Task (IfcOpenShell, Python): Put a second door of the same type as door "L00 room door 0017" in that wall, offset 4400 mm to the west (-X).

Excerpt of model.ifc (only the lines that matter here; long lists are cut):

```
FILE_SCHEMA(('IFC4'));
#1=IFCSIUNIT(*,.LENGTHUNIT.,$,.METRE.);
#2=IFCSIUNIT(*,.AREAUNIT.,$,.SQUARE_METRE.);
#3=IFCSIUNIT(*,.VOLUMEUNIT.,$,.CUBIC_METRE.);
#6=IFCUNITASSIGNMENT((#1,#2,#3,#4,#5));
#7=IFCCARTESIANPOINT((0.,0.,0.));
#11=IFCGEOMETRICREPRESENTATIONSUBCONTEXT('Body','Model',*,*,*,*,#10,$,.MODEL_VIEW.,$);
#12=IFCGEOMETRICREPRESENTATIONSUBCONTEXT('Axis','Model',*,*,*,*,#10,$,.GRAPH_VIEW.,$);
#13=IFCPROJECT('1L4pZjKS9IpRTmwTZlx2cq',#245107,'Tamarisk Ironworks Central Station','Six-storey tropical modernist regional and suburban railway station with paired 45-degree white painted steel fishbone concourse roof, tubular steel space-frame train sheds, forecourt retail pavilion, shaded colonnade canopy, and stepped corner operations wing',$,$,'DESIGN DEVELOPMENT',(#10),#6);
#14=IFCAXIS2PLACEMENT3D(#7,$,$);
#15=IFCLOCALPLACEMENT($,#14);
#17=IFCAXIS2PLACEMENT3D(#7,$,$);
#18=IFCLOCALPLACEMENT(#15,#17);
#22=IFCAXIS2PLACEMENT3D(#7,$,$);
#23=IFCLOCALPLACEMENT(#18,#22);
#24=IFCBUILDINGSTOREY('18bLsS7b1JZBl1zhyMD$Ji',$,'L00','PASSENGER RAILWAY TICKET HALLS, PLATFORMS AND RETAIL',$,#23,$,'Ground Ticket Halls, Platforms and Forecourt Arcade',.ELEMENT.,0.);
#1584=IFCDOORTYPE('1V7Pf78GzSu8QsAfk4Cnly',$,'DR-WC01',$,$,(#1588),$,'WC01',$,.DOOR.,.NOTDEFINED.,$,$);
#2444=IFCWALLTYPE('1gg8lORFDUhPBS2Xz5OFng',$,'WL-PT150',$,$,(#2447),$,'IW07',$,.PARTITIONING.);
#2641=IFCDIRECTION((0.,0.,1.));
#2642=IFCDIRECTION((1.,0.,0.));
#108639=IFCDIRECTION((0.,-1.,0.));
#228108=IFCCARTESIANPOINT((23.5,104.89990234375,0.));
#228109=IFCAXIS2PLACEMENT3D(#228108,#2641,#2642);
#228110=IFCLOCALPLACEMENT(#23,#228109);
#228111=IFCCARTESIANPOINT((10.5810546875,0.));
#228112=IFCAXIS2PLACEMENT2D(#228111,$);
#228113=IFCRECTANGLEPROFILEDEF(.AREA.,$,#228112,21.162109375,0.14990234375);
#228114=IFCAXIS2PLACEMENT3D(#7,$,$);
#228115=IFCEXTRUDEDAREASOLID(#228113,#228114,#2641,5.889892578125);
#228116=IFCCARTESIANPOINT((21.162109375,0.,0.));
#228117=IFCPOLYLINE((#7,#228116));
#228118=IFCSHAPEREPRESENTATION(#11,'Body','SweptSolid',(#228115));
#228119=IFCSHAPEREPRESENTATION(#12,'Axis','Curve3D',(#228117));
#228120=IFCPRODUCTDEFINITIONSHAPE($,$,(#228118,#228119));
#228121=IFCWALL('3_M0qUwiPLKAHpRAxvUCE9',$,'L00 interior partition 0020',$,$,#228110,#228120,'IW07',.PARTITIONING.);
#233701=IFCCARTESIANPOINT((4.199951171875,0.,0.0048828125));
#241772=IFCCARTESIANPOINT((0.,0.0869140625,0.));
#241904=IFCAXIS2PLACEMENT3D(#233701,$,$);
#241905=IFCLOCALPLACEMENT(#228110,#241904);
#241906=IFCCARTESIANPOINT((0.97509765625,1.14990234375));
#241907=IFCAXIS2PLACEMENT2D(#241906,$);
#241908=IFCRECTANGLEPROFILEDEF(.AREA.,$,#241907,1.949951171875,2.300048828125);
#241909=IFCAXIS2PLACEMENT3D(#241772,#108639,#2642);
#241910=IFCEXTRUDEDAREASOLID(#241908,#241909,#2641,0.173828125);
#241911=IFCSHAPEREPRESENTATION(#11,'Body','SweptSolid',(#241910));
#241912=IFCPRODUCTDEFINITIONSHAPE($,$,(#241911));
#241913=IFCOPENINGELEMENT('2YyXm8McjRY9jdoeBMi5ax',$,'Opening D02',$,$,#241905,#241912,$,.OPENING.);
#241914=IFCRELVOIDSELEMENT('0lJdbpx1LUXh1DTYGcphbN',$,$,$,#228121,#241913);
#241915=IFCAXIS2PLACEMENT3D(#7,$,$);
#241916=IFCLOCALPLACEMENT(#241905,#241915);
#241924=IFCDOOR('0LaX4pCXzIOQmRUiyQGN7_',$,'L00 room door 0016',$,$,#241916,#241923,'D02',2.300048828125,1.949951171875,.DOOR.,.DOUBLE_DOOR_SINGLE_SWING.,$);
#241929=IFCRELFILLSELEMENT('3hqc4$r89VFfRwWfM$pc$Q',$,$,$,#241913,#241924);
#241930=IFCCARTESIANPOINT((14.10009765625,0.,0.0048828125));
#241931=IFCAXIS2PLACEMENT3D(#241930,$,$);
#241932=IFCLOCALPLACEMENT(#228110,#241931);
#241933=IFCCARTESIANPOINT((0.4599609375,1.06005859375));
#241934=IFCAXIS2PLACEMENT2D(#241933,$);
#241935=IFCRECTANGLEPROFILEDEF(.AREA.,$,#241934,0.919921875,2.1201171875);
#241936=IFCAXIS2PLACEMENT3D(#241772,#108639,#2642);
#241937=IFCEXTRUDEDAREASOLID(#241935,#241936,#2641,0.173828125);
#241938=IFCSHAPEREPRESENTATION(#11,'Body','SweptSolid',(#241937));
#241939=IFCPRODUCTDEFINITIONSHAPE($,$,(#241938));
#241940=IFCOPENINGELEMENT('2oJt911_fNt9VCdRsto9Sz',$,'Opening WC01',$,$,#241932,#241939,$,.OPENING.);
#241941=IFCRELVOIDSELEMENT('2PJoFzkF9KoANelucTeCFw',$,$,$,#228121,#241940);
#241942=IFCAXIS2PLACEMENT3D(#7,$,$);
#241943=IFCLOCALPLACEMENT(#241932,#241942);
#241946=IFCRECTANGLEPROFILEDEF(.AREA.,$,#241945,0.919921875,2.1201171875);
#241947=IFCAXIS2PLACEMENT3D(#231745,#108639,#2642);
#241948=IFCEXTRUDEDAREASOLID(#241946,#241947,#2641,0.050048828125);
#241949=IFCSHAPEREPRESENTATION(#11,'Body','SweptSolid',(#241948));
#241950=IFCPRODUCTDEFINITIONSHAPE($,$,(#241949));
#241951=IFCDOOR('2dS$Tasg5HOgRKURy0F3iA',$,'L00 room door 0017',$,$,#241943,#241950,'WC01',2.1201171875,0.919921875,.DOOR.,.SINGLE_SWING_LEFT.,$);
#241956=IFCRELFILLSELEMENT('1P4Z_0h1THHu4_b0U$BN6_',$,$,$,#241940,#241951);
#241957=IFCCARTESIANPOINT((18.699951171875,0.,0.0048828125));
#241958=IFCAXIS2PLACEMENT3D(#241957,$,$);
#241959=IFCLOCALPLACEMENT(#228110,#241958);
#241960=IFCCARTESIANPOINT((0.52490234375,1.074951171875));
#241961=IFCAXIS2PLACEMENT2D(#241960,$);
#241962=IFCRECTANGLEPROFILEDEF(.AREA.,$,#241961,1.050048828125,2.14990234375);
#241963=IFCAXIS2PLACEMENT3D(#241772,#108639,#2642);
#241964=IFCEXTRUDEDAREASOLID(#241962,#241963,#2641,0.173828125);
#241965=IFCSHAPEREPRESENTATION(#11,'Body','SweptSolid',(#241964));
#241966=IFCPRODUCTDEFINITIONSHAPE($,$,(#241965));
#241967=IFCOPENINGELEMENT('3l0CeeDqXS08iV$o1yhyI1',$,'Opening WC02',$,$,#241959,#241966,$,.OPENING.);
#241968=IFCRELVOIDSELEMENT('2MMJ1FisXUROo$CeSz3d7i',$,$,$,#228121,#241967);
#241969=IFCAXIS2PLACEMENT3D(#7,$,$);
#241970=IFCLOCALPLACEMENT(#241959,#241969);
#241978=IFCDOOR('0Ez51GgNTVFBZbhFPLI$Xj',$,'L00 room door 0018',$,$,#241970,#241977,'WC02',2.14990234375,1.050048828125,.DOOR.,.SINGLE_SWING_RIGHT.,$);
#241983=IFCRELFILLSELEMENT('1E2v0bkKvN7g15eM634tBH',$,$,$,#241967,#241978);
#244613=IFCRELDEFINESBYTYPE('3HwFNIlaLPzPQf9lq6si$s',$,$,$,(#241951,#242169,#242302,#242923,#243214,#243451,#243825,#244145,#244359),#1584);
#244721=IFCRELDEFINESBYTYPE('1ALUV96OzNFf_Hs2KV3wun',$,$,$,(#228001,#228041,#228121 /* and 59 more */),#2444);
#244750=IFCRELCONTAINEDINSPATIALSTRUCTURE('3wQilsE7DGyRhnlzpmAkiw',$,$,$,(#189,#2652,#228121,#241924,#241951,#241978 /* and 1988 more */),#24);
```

```python
import ifcopenshell
import ifcopenshell.api.feature
import ifcopenshell.api.geometry
import ifcopenshell.api.root
import ifcopenshell.geom
import ifcopenshell.util.element
import ifcopenshell.util.placement
import ifcopenshell.util.shape

model = ifcopenshell.open("model.ifc")
settings = ifcopenshell.geom.settings()


def volume(element):
    """Net volume in cubic metres, openings subtracted."""
    shape = ifcopenshell.geom.create_shape(settings, element)
    return ifcopenshell.util.shape.get_volume(shape.geometry)


door = model.by_id(241951)
opening = door.FillsVoids[0].RelatingOpeningElement
wall = opening.VoidsElements[0].RelatingBuildingElement
before = volume(wall)
shift = ifcopenshell.util.placement.get_local_placement(wall.ObjectPlacement)[:3, 0] * -4.4

# copy_class copies the void relationship, type, container and properties, but no geometry.
new_opening = ifcopenshell.api.root.copy_class(model, product=opening)
new_opening.Representation = ifcopenshell.util.element.copy_deep(
    model, opening.Representation, exclude=["IfcGeometricRepresentationContext", "IfcRepresentationMap"]
)
new_door = ifcopenshell.api.root.copy_class(model, product=door)
new_door.Representation = ifcopenshell.util.element.copy_deep(
    model, door.Representation, exclude=["IfcGeometricRepresentationContext", "IfcRepresentationMap"]
)
new_door.Tag = None
ifcopenshell.api.feature.add_filling(model, opening=new_opening, element=new_door)

for old, new in ((opening, new_opening), (door, new_door)):
    matrix = ifcopenshell.util.placement.get_local_placement(old.ObjectPlacement)
    matrix[:3, 3] += shift
    ifcopenshell.api.geometry.edit_object_placement(model, product=new, matrix=matrix, is_si=False)

after = volume(wall)

print(f"wall volume {before:.3f} -> {after:.3f} m3")

model.write("model-out.ifc")
```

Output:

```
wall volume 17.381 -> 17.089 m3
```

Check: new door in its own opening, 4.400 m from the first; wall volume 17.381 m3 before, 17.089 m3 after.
